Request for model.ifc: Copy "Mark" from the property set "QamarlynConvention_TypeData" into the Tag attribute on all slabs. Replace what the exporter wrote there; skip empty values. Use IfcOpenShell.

First a look at what the model holds.

```python
import ifcopenshell
import ifcopenshell.util.element

model = ifcopenshell.open("model.ifc")
print(model.schema)
slabs = model.by_type("IfcSlab")
print(len(slabs), "slabs")
for e in slabs[:8]:
    source = ifcopenshell.util.element.get_pset(e, "QamarlynConvention_TypeData", "Mark")
    target = e.Tag
    print(e.id(), repr(source), repr(target), sep=" | ")
```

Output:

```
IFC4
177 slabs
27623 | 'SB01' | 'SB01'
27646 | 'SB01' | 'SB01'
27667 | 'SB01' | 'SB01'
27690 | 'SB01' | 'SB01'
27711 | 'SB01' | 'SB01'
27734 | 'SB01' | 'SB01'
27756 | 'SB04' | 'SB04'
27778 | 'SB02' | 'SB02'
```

```python
import ifcopenshell
import ifcopenshell.util.element

model = ifcopenshell.open("model.ifc")

count = 0
for e in model.by_type("IfcSlab"):
    value = ifcopenshell.util.element.get_pset(e, "QamarlynConvention_TypeData", "Mark")
    current = e.Tag
    if not value or not value.strip() or current == value:
        continue
    e.Tag = value
    count += 1

print(count, "slabs updated")

model.write("model_edited.ifc")
```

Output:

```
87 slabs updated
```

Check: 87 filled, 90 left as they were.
